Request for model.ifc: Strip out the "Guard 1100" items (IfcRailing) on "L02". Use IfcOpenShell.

First a look at what the model holds.

```python
import ifcopenshell
import ifcopenshell.util.element

model = ifcopenshell.open("model.ifc")
print(model.schema)
storey = next(s for s in model.by_type("IfcBuildingStorey") if s.Name == "L02")
railings = [e for e in ifcopenshell.util.element.get_decomposition(storey) if e.is_a("IfcRailing")]
seen = {}
for e in railings:
    element_type = ifcopenshell.util.element.get_type(e)
    name = element_type.Name if element_type not in (None, e) else None
    seen[name] = seen.get(name, 0) + 1
for name, count in sorted(seen.items(), key=str):
    print(count, "x", name)
```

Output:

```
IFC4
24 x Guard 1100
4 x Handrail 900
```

```python
import ifcopenshell
import ifcopenshell.api.root
import ifcopenshell.util.element

model = ifcopenshell.open("model.ifc")

storey = next(s for s in model.by_type("IfcBuildingStorey") if s.Name == "L02")
railings = [e for e in ifcopenshell.util.element.get_decomposition(storey) if e.is_a("IfcRailing")]
targets = [e for e in railings if (t := ifcopenshell.util.element.get_type(e)) not in (None, e) and t.Name == "Guard 1100"]

for e in targets:
    ifcopenshell.api.root.remove_product(model, product=e)
print(len(targets), "removed")

model.write("model_edited.ifc")
```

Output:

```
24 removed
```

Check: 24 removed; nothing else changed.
